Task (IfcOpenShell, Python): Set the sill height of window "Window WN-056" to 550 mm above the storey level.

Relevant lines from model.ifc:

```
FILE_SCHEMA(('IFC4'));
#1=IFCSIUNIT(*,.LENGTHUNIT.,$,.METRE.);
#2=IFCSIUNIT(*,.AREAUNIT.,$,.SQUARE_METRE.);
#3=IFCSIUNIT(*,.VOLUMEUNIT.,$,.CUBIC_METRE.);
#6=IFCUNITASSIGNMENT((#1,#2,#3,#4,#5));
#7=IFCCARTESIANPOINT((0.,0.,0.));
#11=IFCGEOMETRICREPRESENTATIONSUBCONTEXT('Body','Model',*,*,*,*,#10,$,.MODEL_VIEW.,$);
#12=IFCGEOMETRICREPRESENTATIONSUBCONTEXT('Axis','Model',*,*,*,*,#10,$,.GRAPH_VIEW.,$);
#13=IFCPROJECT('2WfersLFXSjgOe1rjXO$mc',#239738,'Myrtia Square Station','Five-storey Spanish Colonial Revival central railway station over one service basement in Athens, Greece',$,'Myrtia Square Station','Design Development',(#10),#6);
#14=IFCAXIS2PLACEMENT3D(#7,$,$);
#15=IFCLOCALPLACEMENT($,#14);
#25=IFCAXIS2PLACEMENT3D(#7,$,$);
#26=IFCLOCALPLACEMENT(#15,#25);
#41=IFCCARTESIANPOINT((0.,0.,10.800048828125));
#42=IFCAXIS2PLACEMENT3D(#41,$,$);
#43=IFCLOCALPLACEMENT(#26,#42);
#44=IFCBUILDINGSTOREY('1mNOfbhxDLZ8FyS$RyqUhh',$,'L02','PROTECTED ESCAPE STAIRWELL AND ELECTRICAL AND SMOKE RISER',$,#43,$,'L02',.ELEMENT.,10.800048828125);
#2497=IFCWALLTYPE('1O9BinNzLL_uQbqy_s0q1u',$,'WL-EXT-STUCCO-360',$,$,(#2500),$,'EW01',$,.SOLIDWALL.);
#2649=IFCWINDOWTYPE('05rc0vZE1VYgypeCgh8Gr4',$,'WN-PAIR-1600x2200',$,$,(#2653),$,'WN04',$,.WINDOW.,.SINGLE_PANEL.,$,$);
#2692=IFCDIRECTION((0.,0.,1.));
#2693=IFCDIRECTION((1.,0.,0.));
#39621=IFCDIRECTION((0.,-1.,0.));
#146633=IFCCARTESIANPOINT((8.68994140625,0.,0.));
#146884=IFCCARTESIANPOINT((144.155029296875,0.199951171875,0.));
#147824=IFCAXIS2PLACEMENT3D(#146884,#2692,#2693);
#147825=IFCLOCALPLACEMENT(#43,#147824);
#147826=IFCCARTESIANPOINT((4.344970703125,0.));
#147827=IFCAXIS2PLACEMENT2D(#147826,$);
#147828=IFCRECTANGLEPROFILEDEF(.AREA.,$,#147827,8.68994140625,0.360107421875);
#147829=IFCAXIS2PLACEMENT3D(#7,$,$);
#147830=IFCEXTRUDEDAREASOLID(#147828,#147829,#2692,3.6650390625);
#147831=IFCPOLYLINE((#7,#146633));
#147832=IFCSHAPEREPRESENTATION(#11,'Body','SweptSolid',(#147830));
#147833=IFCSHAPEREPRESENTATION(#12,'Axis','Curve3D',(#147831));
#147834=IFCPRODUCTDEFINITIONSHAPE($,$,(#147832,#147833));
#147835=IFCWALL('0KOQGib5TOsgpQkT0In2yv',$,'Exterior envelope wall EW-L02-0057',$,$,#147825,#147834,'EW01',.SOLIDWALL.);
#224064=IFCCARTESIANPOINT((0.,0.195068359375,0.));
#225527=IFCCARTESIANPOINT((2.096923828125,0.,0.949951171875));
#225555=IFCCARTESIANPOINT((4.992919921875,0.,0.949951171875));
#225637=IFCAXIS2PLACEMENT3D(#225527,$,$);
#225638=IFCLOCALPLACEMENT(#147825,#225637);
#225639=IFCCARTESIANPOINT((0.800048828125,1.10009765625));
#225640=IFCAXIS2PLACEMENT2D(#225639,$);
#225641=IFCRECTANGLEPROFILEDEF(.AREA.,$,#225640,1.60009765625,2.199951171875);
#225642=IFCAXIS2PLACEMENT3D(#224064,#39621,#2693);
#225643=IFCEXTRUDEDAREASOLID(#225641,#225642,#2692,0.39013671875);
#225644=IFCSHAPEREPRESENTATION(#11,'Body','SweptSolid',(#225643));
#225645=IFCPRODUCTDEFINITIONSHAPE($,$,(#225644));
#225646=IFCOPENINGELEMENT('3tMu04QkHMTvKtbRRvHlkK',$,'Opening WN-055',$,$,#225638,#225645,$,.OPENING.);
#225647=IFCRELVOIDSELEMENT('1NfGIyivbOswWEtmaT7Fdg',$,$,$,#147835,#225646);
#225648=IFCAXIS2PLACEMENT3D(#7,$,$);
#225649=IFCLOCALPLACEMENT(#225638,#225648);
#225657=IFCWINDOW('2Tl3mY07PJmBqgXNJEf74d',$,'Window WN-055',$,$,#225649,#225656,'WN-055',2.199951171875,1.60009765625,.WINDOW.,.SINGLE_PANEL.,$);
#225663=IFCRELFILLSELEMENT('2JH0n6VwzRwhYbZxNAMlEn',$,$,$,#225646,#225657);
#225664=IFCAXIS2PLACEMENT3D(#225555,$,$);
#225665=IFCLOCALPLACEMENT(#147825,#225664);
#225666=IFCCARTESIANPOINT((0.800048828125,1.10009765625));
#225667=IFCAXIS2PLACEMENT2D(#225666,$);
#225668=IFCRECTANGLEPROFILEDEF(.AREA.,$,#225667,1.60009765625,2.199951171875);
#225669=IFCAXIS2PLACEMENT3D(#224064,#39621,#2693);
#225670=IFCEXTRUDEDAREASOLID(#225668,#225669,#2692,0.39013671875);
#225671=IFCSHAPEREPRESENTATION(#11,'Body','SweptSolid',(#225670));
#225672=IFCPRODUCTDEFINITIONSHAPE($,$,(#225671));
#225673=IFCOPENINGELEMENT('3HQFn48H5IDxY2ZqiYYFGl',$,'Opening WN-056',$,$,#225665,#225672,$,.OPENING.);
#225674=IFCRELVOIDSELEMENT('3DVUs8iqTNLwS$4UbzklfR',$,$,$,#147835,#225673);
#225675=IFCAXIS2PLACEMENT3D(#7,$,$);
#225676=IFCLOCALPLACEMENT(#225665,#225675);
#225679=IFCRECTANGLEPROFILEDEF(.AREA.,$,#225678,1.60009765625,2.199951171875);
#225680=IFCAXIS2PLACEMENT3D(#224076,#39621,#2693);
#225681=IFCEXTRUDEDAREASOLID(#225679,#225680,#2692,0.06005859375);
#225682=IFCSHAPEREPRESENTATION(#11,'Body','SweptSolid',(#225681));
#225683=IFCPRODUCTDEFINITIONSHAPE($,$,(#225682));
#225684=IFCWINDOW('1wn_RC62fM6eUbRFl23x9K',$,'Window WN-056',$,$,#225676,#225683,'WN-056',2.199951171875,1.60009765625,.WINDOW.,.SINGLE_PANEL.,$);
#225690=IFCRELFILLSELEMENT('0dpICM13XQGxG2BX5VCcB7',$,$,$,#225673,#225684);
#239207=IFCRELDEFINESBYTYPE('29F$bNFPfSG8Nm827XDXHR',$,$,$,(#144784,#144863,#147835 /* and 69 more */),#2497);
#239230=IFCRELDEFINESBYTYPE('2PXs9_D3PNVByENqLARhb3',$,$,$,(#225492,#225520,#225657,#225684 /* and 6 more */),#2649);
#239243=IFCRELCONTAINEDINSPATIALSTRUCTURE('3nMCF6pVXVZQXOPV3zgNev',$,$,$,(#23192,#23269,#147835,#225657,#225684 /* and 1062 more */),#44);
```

```python
import numpy as np
import ifcopenshell
import ifcopenshell.api.geometry
import ifcopenshell.geom
import ifcopenshell.util.element
import ifcopenshell.util.placement
import ifcopenshell.util.shape
import ifcopenshell.util.unit

model = ifcopenshell.open("model.ifc")
unit_scale = ifcopenshell.util.unit.calculate_unit_scale(model)

window = model.by_guid("1wn_RC62fM6eUbRFl23x9K")
opening = window.FillsVoids[0].RelatingOpeningElement
storey = ifcopenshell.util.element.get_container(window, ifc_class="IfcBuildingStorey")
level = ifcopenshell.util.placement.get_local_placement(storey.ObjectPlacement)[2, 3]

# The opening's origin need not be at the sill, so measure its lowest point.
shape = ifcopenshell.geom.create_shape(ifcopenshell.geom.settings(), opening)
bottom = ifcopenshell.util.shape.get_shape_bottom_elevation(shape, shape.geometry) / unit_scale
dz = level + 0.55 - bottom

shift = np.array([0.0, 0.0, dz])
# The window is placed relative to its opening, so it follows when the opening moves.
matrix = ifcopenshell.util.placement.get_local_placement(opening.ObjectPlacement)
matrix[:3, 3] += shift
ifcopenshell.api.geometry.edit_object_placement(
    model, product=opening, matrix=matrix, is_si=False, should_transform_children=True
)

print(f"moved by {dz * unit_scale:+.3f} m")

model.write("model_updated.ifc")
```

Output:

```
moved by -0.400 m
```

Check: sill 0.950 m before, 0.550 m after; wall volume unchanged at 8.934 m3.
